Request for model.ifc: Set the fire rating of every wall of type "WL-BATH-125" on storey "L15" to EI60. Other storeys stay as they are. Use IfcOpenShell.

First a look at what the model holds.

```python
import ifcopenshell
import ifcopenshell.util.element

model = ifcopenshell.open("model.ifc")
print(model.schema)
storey = next(s for s in model.by_type("IfcBuildingStorey") if s.Name == "L15")
walls = [e for e in ifcopenshell.util.element.get_decomposition(storey) if e.is_a("IfcWall")]
seen = {}
for e in walls:
    element_type = ifcopenshell.util.element.get_type(e)
    key = (element_type.Name if element_type != e and element_type else None, ifcopenshell.util.element.get_pset(e, "Pset_WallCommon", "FireRating"))
    seen[key] = seen.get(key, 0) + 1
for (name, value), count in sorted(seen.items(), key=str):
    print(count, "x", name, "|", value)
```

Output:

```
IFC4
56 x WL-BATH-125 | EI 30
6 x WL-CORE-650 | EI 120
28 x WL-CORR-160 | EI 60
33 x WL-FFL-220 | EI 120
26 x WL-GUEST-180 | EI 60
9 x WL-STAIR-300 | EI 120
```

```python
import ifcopenshell
import ifcopenshell.api.pset
import ifcopenshell.util.element

model = ifcopenshell.open("model.ifc")

storey = next(s for s in model.by_type("IfcBuildingStorey") if s.Name == "L15")
walls = [e for e in ifcopenshell.util.element.get_decomposition(storey) if e.is_a("IfcWall")]

count = 0
for e in walls:
    element_type = ifcopenshell.util.element.get_type(e)
    if element_type in (None, e) or element_type.Name != "WL-BATH-125":
        continue
    # add_pset returns the element's existing set when there is one.
    pset = ifcopenshell.api.pset.add_pset(model, product=e, name="Pset_WallCommon")
    ifcopenshell.api.pset.edit_pset(model, pset=pset, properties={"FireRating": "EI60"})
    count += 1

print(count, "walls updated")

model.write("model-out.ifc")
```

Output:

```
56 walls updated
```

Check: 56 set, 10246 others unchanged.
